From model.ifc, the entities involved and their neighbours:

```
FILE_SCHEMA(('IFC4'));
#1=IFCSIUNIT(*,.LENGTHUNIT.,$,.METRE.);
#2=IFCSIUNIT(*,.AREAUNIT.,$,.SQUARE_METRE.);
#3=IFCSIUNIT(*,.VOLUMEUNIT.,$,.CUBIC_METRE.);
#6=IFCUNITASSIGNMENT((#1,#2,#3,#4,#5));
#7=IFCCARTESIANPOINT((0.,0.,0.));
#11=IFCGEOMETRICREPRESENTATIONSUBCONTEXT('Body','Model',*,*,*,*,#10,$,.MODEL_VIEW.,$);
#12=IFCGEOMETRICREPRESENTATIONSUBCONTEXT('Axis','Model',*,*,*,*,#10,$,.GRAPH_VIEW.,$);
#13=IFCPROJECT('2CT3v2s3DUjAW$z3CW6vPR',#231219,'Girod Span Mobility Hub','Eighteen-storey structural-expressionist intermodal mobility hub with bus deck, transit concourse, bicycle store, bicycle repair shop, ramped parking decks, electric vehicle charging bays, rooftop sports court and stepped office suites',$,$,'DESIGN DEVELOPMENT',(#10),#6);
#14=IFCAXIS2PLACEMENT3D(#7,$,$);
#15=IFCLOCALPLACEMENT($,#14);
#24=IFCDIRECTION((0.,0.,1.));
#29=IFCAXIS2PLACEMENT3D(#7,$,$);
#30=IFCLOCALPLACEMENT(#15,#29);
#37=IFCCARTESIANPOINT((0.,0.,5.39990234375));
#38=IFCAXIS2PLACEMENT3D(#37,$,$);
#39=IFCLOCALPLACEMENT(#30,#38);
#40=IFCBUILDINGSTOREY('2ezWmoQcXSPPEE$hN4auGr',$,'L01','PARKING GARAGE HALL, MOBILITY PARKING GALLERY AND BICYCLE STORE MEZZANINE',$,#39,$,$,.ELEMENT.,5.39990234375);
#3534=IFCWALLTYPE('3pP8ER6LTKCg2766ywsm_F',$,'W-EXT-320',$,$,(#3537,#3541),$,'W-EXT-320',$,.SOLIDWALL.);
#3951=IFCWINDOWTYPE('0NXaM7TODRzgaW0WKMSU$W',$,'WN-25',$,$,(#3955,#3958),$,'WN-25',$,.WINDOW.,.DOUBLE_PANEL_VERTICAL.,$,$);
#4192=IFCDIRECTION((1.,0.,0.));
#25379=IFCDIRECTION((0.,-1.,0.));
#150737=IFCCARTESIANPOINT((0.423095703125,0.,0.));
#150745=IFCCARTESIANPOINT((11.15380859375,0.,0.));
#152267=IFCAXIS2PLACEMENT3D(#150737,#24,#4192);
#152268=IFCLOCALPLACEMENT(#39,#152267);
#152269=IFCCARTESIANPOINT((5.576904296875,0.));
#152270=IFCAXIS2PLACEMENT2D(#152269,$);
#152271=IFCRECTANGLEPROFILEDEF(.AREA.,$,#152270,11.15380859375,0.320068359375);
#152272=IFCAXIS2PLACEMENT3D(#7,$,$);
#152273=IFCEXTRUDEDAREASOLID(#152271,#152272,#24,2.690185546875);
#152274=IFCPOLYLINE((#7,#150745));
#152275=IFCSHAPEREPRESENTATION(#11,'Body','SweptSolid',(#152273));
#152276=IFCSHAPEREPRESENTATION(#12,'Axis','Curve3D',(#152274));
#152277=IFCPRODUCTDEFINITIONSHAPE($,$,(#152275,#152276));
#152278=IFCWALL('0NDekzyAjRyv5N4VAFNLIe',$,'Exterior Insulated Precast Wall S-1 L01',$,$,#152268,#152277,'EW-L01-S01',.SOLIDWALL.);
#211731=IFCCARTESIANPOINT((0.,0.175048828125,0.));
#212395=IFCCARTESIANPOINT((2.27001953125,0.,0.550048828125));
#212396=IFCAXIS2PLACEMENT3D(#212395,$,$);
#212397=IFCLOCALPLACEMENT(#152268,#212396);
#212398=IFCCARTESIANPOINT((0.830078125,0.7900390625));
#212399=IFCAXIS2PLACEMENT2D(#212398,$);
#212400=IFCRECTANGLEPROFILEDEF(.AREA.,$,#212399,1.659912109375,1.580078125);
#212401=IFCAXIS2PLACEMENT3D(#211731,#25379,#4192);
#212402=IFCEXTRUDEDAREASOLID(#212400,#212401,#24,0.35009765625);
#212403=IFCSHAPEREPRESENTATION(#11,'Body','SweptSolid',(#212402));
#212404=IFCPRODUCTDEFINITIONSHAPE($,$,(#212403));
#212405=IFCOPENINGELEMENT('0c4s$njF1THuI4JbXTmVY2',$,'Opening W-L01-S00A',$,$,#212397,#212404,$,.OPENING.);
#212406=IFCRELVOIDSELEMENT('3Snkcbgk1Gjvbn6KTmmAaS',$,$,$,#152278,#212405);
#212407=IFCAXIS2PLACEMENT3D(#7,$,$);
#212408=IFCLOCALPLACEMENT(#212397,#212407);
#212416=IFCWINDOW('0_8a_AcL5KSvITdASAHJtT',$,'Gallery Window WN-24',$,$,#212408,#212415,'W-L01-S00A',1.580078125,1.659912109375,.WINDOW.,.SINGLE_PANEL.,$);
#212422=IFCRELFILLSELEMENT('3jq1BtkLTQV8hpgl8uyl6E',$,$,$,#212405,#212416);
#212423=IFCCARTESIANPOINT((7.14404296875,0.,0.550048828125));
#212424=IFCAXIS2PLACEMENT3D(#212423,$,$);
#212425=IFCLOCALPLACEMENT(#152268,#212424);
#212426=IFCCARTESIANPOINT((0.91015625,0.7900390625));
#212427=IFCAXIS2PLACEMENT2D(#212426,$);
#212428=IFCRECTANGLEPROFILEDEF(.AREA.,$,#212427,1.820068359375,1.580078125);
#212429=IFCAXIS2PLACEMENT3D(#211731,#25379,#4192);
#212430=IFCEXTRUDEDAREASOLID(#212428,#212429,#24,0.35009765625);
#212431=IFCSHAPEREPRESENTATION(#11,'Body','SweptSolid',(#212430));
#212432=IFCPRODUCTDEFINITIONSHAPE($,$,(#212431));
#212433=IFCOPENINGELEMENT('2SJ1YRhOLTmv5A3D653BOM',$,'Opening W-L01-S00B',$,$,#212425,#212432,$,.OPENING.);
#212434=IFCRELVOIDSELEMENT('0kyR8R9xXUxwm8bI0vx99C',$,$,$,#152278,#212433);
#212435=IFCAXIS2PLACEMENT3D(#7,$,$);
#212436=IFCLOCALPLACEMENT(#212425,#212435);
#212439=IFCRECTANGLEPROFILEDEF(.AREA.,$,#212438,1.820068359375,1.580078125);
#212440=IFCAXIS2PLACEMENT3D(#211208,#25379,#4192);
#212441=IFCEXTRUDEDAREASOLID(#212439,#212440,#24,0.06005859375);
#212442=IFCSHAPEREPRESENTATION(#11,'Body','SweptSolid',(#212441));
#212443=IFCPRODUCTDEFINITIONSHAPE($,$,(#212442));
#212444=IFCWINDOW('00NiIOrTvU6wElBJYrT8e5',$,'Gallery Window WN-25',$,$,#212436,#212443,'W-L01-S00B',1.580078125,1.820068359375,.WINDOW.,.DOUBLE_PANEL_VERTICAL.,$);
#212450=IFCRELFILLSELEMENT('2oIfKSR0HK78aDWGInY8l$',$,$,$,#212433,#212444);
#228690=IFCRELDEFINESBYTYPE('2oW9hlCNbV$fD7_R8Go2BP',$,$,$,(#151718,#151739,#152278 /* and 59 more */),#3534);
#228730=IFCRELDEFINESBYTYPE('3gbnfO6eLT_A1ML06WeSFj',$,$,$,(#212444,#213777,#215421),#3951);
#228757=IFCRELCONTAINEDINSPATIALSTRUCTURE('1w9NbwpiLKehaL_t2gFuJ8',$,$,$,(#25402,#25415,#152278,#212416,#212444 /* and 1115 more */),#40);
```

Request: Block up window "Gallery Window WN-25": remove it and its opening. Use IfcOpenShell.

```python
import ifcopenshell
import ifcopenshell.api.feature
import ifcopenshell.api.root
import ifcopenshell.geom
import ifcopenshell.util.shape

model = ifcopenshell.open("model.ifc")
settings = ifcopenshell.geom.settings()


def volume(element):
    """Net volume in cubic metres, openings subtracted."""
    shape = ifcopenshell.geom.create_shape(settings, element)
    return ifcopenshell.util.shape.get_volume(shape.geometry)


window = model.by_id(212444)
opening = window.FillsVoids[0].RelatingOpeningElement
wall = opening.VoidsElements[0].RelatingBuildingElement
before = volume(wall)

ifcopenshell.api.root.remove_product(model, product=window)
ifcopenshell.api.feature.remove_feature(model, feature=opening)

after = volume(wall)

print(f"wall volume {before:.3f} -> {after:.3f} m3")

model.write("model_v2.ifc")
```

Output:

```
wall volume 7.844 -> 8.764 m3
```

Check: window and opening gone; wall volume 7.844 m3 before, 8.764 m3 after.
